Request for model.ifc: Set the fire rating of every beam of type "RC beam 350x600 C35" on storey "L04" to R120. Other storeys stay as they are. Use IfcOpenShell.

First a look at what the model holds.

```python
import ifcopenshell
import ifcopenshell.util.element

model = ifcopenshell.open("model.ifc")
print(model.schema)
storey = next(s for s in model.by_type("IfcBuildingStorey") if s.Name == "L04")
beams = [e for e in ifcopenshell.util.element.get_decomposition(storey) if e.is_a("IfcBeam")]
seen = {}
for e in beams:
    element_type = ifcopenshell.util.element.get_type(e)
    key = (element_type.Name if element_type != e and element_type else None, ifcopenshell.util.element.get_pset(e, "Pset_BeamCommon", "FireRating"))
    seen[key] = seen.get(key, 0) + 1
for (name, value), count in sorted(seen.items(), key=str):
    print(count, "x", name, "|", value)
```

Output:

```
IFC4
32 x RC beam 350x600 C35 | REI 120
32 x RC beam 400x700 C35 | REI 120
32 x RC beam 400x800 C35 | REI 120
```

```python
import ifcopenshell
import ifcopenshell.api.pset
import ifcopenshell.util.element

model = ifcopenshell.open("model.ifc")

storey = next(s for s in model.by_type("IfcBuildingStorey") if s.Name == "L04")
beams = [e for e in ifcopenshell.util.element.get_decomposition(storey) if e.is_a("IfcBeam")]

count = 0
for e in beams:
    element_type = ifcopenshell.util.element.get_type(e)
    if element_type in (None, e) or element_type.Name != "RC beam 350x600 C35":
        continue
    # add_pset returns the element's existing set when there is one.
    pset = ifcopenshell.api.pset.add_pset(model, product=e, name="Pset_BeamCommon")
    ifcopenshell.api.pset.edit_pset(model, pset=pset, properties={"FireRating": "R120"})
    count += 1

print(count, "beams updated")

model.write("model_v2.ifc")
```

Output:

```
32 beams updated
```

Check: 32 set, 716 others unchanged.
